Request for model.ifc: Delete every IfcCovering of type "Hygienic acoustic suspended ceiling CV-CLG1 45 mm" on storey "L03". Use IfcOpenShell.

First a look at what the model holds.

```python
import ifcopenshell
import ifcopenshell.util.element

model = ifcopenshell.open("model.ifc")
print(model.schema)
storey = next(s for s in model.by_type("IfcBuildingStorey") if s.Name == "L03")
coverings = [e for e in ifcopenshell.util.element.get_decomposition(storey) if e.is_a("IfcCovering")]
seen = {}
for e in coverings:
    element_type = ifcopenshell.util.element.get_type(e)
    name = element_type.Name if element_type not in (None, e) else None
    seen[name] = seen.get(name, 0) + 1
for name, count in sorted(seen.items(), key=str):
    print(count, "x", name)
```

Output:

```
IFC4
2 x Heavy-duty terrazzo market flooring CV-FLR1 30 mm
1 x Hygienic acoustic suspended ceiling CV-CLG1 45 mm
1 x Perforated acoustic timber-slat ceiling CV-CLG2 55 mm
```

```python
import ifcopenshell
import ifcopenshell.api.root
import ifcopenshell.util.element

model = ifcopenshell.open("model.ifc")

storey = next(s for s in model.by_type("IfcBuildingStorey") if s.Name == "L03")
coverings = [e for e in ifcopenshell.util.element.get_decomposition(storey) if e.is_a("IfcCovering")]
targets = [e for e in coverings if (t := ifcopenshell.util.element.get_type(e)) not in (None, e) and t.Name == "Hygienic acoustic suspended ceiling CV-CLG1 45 mm"]

for e in targets:
    ifcopenshell.api.root.remove_product(model, product=e)
print(len(targets), "removed")

model.write("model_rev.ifc")
```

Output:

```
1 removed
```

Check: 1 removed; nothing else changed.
